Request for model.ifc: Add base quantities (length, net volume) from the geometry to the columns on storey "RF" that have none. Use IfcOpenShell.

First a look at what the model holds.

```python
import ifcopenshell
import ifcopenshell.util.element
import ifcopenshell.util.unit

model = ifcopenshell.open("model.ifc")
print(model.schema)
for unit_type in ("LENGTHUNIT", "AREAUNIT", "VOLUMEUNIT"):
    print(unit_type, ifcopenshell.util.unit.calculate_unit_scale(model, unit_type))
storey = next(s for s in model.by_type("IfcBuildingStorey") if s.Name == "RF")
columns = [e for e in ifcopenshell.util.element.get_decomposition(storey) if e.is_a("IfcColumn")]
for e in sorted(columns, key=lambda e: e.id()):
    print(e.id(), e.is_a(), e.Name, list(ifcopenshell.util.element.get_psets(e, qtos_only=True)), sep=" | ")
```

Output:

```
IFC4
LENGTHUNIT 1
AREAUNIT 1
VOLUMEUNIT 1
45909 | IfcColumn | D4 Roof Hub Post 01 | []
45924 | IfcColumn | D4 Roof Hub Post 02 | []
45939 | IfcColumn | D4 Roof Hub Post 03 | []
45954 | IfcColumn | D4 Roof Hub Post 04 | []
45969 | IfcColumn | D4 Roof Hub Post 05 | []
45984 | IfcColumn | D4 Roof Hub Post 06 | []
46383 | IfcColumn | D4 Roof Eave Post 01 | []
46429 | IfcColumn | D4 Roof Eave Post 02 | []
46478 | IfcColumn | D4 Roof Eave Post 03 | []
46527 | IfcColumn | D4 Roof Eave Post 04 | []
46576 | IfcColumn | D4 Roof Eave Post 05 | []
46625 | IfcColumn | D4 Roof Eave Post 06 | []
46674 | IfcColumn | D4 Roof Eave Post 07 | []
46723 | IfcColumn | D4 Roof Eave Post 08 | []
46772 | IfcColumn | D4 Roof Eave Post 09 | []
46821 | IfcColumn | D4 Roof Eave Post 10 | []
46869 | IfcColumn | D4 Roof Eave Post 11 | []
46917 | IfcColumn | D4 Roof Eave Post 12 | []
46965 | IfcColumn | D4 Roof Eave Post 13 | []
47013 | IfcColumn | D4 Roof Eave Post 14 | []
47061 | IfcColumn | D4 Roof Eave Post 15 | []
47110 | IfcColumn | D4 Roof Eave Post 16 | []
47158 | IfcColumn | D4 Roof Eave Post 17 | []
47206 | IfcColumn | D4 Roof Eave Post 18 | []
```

```python
import ifcopenshell
import ifcopenshell.api.pset
import ifcopenshell.geom
import ifcopenshell.util.element
import ifcopenshell.util.shape
import ifcopenshell.util.unit

model = ifcopenshell.open("model.ifc")
unit_scale = ifcopenshell.util.unit.calculate_unit_scale(model)
volume_scale = ifcopenshell.util.unit.calculate_unit_scale(model, "VOLUMEUNIT")
settings = ifcopenshell.geom.settings()

storey = next(s for s in model.by_type("IfcBuildingStorey") if s.Name == "RF")
columns = [e for e in ifcopenshell.util.element.get_decomposition(storey) if e.is_a("IfcColumn")]

for e in sorted(columns, key=lambda e: e.id()):
    if ifcopenshell.util.element.get_psets(e, qtos_only=True, should_inherit=False):
        continue
    # Geometry comes back in metres, in the element's own axes.
    shape = ifcopenshell.geom.create_shape(settings, e)
    values = {
        "Length": ifcopenshell.util.shape.get_z(shape.geometry) / unit_scale,
        "NetVolume": ifcopenshell.util.shape.get_volume(shape.geometry) / volume_scale,
    }
    qto = ifcopenshell.api.pset.add_qto(model, product=e, name="Qto_ColumnBaseQuantities")
    ifcopenshell.api.pset.edit_qto(model, qto=qto, properties=values)
    print(e.id(), {k: round(v, 3) for k, v in values.items()})

model.write("model-out.ifc")
```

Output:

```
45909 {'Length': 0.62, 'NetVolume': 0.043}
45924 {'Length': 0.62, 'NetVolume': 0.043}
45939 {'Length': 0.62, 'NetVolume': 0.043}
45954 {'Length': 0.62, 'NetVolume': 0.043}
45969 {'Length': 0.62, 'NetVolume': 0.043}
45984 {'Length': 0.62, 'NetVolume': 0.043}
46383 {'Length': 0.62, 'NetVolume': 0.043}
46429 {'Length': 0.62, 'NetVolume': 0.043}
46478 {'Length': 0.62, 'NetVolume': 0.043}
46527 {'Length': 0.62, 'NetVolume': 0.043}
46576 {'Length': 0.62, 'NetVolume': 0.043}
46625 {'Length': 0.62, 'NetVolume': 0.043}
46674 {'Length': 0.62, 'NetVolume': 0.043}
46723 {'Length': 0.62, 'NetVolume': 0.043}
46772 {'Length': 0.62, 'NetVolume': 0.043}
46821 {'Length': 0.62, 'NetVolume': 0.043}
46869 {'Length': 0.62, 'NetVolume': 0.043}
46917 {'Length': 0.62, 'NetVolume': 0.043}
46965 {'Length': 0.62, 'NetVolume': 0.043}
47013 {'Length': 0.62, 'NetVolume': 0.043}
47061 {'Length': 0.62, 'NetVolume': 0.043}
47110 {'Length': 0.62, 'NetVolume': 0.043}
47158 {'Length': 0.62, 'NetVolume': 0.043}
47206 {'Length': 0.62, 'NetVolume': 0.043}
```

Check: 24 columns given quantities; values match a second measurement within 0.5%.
